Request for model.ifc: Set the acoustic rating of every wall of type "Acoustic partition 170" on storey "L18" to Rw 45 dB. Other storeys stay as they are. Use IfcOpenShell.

First a look at what the model holds.

```python
import ifcopenshell
import ifcopenshell.util.element

model = ifcopenshell.open("model.ifc")
print(model.schema)
storey = next(s for s in model.by_type("IfcBuildingStorey") if s.Name == "L18")
walls = [e for e in ifcopenshell.util.element.get_decomposition(storey) if e.is_a("IfcWall")]
seen = {}
for e in walls:
    element_type = ifcopenshell.util.element.get_type(e)
    key = (element_type.Name if element_type != e and element_type else None, ifcopenshell.util.element.get_pset(e, "Pset_WallCommon", "AcousticRating"))
    seen[key] = seen.get(key, 0) + 1
for (name, value), count in sorted(seen.items(), key=str):
    print(count, "x", name, "|", value)
```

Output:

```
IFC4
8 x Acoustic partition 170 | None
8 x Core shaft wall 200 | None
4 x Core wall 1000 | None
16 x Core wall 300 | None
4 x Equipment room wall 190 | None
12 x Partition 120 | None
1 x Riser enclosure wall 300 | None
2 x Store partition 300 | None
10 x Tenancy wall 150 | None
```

```python
import ifcopenshell
import ifcopenshell.api.pset
import ifcopenshell.util.element

model = ifcopenshell.open("model.ifc")

storey = next(s for s in model.by_type("IfcBuildingStorey") if s.Name == "L18")
walls = [e for e in ifcopenshell.util.element.get_decomposition(storey) if e.is_a("IfcWall")]

count = 0
for e in walls:
    element_type = ifcopenshell.util.element.get_type(e)
    if element_type in (None, e) or element_type.Name != "Acoustic partition 170":
        continue
    found = ifcopenshell.util.element.get_pset(e, "Pset_WallCommon", should_inherit=False)
    if found:
        pset = model.by_id(found["id"])
        if len(ifcopenshell.util.element.get_elements_by_pset(pset)) > 1:
            pset = ifcopenshell.api.pset.unshare_pset(model, products=[e], pset=pset)[0]
    else:
        pset = ifcopenshell.api.pset.add_pset(model, product=e, name="Pset_WallCommon")
    ifcopenshell.api.pset.edit_pset(model, pset=pset, properties={"AcousticRating": "Rw 45 dB"})
    count += 1

print(count, "walls updated")

model.write("model_edited.ifc")
```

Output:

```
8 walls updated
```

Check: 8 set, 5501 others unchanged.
